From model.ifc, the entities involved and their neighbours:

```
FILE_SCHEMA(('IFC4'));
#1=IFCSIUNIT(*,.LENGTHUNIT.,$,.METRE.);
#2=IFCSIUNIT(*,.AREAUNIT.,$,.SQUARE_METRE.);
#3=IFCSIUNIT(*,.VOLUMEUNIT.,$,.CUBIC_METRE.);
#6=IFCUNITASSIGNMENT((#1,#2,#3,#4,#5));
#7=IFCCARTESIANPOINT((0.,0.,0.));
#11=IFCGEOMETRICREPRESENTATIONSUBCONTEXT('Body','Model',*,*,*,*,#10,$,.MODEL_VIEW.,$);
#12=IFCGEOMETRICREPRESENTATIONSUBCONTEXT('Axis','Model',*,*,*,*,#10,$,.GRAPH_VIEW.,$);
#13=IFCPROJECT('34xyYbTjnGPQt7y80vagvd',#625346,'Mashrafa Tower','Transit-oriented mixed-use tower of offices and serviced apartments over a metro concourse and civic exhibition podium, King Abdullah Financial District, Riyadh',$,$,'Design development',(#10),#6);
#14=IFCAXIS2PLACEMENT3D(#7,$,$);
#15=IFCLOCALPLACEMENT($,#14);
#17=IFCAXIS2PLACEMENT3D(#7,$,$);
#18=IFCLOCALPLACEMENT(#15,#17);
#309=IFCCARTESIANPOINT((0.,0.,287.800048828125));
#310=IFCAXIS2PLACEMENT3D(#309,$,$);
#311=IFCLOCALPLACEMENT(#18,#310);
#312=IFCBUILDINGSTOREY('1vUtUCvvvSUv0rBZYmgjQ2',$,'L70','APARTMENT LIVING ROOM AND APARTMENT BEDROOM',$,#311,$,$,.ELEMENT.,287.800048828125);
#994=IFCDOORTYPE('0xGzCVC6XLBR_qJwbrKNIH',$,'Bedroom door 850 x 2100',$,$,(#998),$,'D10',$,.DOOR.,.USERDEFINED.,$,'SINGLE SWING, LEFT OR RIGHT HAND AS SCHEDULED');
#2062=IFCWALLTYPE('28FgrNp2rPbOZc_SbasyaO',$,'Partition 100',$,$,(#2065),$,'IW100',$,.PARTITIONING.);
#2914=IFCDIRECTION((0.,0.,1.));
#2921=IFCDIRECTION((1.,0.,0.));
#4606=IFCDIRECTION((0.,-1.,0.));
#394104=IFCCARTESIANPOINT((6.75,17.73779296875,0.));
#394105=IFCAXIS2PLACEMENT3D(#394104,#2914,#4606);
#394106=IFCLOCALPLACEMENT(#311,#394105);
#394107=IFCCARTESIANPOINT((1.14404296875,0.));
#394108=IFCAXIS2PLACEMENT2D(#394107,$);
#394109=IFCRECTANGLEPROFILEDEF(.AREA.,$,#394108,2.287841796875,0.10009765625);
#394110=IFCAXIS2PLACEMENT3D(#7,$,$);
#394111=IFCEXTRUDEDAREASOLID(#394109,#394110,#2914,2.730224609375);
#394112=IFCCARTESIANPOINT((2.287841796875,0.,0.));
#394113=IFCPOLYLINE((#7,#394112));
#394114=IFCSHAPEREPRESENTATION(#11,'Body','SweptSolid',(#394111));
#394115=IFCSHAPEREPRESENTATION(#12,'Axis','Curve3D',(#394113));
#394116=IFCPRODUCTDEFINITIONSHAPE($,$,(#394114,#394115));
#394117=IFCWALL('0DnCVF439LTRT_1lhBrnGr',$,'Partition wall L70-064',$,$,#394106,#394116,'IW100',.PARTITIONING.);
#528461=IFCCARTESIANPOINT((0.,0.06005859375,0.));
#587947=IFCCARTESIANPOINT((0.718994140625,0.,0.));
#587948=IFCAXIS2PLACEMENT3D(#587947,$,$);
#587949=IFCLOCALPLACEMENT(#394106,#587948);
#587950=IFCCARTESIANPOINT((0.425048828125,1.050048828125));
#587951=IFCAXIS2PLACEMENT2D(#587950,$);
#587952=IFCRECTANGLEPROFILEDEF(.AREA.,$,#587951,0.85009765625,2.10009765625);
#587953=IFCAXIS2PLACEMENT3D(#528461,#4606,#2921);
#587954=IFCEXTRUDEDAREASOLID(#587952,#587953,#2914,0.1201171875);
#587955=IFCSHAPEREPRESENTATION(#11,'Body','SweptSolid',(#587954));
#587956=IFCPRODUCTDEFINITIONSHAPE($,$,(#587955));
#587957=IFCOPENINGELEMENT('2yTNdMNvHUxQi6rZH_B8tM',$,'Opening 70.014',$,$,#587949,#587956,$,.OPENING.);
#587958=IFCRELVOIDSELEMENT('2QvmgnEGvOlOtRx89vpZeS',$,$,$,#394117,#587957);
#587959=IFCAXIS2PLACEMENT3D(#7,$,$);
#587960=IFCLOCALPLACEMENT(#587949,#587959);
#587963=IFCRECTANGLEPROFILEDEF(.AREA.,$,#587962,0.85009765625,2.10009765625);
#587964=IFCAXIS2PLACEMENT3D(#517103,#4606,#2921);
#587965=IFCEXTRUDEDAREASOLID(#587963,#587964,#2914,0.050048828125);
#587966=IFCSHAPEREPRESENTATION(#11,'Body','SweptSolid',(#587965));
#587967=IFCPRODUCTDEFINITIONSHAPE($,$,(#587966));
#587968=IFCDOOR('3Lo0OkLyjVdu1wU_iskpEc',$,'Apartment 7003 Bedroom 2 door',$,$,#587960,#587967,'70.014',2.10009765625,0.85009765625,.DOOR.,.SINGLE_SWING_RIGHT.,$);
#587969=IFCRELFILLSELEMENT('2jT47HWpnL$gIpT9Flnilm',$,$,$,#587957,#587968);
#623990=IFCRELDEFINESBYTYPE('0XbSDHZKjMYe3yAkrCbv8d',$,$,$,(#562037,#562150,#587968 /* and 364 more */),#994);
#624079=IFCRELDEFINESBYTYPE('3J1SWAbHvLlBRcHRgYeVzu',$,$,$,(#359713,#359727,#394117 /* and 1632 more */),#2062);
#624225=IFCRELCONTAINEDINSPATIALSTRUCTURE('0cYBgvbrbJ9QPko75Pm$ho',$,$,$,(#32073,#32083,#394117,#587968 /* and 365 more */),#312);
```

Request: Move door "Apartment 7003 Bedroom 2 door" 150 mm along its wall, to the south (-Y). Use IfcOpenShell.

```python
import ifcopenshell
import ifcopenshell.api.geometry
import ifcopenshell.util.placement
import ifcopenshell.util.unit

model = ifcopenshell.open("model.ifc")
unit_scale = ifcopenshell.util.unit.calculate_unit_scale(model)

door = model.by_guid("3Lo0OkLyjVdu1wU_iskpEc")
opening = door.FillsVoids[0].RelatingOpeningElement
wall = opening.VoidsElements[0].RelatingBuildingElement

wall_matrix = ifcopenshell.util.placement.get_local_placement(wall.ObjectPlacement)
shift = wall_matrix[:3, 0] * 0.15 / unit_scale
before = ifcopenshell.util.placement.get_local_placement(door.ObjectPlacement)[:3, 3].copy()

# The door is placed relative to its opening, so it follows when the opening moves.
matrix = ifcopenshell.util.placement.get_local_placement(opening.ObjectPlacement)
matrix[:3, 3] += shift
ifcopenshell.api.geometry.edit_object_placement(
    model, product=opening, matrix=matrix, is_si=False, should_transform_children=True
)

after = ifcopenshell.util.placement.get_local_placement(door.ObjectPlacement)[:3, 3]
print("door moved by", (after - before).round(3) + 0.0)

model.write("model_edited.ifc")
```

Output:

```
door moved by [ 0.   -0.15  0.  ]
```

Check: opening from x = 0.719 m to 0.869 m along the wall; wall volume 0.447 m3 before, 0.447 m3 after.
